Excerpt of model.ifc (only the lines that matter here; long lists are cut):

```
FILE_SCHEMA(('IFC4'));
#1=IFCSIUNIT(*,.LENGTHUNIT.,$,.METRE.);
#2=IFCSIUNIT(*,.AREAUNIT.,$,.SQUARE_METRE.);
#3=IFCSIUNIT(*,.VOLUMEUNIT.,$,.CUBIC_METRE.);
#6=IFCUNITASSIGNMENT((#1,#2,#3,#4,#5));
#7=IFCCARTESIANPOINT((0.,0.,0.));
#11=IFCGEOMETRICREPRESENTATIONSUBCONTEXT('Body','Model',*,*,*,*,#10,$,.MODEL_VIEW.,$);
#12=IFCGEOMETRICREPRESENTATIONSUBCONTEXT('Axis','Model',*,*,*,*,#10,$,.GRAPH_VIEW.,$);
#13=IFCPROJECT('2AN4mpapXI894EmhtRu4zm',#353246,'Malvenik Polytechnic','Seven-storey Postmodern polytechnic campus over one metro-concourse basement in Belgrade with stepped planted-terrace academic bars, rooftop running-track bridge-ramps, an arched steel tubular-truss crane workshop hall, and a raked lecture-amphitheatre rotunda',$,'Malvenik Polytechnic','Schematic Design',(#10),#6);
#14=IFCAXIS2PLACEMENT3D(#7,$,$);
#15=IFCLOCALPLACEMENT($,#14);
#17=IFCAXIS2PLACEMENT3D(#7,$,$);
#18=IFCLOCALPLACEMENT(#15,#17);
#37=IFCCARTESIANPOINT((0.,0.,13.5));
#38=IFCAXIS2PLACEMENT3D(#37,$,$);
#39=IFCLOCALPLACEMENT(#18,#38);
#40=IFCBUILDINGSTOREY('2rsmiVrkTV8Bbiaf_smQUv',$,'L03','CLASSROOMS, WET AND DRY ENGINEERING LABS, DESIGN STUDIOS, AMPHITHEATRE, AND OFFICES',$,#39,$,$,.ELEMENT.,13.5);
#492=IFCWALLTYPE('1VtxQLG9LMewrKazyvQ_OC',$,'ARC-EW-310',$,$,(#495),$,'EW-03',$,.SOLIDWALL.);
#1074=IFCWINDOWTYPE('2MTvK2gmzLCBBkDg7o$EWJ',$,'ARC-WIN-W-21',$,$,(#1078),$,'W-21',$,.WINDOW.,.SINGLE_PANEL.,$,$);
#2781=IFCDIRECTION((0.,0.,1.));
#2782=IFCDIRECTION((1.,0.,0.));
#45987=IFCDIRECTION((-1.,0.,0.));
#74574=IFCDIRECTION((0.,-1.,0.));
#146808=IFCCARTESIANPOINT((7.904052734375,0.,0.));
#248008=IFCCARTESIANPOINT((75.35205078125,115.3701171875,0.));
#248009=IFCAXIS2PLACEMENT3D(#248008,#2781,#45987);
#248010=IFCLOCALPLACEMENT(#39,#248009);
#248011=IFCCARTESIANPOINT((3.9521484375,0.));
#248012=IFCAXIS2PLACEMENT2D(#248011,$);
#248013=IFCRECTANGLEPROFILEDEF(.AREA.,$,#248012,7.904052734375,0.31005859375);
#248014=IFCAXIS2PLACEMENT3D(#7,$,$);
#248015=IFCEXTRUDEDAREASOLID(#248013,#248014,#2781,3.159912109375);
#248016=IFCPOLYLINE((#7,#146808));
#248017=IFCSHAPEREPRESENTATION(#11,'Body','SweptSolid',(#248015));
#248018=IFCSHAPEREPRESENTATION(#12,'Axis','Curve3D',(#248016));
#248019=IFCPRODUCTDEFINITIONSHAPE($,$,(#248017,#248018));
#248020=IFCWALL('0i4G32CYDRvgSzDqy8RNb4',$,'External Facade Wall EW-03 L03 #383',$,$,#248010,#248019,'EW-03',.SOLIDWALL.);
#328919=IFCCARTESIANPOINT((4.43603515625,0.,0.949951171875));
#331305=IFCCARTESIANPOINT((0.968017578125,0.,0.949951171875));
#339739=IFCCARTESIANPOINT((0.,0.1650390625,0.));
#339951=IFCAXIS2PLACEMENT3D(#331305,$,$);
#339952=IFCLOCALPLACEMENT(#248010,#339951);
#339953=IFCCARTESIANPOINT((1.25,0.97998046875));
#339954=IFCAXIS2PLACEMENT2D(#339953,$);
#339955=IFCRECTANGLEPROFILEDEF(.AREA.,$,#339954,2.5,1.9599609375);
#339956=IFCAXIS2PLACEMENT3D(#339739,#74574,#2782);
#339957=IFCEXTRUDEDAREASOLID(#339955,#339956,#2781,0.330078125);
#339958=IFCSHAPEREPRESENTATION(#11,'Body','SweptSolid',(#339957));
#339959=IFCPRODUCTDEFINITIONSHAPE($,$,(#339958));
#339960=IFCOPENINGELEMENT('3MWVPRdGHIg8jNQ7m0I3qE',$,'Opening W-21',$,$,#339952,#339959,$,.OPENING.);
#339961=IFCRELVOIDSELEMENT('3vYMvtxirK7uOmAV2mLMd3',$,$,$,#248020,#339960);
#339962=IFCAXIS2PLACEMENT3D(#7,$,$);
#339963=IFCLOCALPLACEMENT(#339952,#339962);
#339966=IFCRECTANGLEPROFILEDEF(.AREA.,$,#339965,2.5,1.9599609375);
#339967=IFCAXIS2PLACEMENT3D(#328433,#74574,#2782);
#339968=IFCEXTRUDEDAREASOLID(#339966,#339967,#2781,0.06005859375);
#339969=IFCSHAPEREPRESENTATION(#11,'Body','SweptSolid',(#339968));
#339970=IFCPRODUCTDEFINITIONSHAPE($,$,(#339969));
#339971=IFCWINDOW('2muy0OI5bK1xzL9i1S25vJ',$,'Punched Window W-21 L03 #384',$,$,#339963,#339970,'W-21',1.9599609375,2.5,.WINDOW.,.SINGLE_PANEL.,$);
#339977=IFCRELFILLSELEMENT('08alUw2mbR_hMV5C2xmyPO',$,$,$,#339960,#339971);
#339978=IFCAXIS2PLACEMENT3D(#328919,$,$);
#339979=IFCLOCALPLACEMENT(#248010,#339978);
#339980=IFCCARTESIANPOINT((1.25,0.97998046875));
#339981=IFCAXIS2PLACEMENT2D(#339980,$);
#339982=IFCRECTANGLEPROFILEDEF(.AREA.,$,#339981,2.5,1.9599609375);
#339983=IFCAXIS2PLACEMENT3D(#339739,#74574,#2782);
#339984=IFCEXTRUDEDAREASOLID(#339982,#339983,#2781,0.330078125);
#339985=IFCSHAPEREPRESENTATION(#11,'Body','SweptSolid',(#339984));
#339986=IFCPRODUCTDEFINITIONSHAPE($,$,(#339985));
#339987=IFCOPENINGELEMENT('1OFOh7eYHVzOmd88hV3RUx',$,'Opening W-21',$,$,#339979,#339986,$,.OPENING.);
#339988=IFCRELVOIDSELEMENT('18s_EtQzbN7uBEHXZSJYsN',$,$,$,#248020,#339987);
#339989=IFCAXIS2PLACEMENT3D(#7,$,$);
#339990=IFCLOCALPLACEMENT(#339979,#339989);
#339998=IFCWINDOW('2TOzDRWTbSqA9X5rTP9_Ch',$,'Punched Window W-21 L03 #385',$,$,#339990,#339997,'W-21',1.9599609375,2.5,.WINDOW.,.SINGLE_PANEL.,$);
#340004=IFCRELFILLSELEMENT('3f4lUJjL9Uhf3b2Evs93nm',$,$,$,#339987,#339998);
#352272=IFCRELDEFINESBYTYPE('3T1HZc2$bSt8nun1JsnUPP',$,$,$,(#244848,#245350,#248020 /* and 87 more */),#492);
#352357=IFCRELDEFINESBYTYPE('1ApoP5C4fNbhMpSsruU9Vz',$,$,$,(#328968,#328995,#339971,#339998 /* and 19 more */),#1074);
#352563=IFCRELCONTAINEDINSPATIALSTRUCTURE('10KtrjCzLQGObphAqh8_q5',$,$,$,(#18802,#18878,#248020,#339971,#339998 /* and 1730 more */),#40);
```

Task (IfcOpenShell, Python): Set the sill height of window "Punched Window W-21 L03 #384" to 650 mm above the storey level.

```python
import numpy as np
import ifcopenshell
import ifcopenshell.api.geometry
import ifcopenshell.geom
import ifcopenshell.util.element
import ifcopenshell.util.placement
import ifcopenshell.util.shape
import ifcopenshell.util.unit

model = ifcopenshell.open("model.ifc")
unit_scale = ifcopenshell.util.unit.calculate_unit_scale(model)

window = model.by_guid("2muy0OI5bK1xzL9i1S25vJ")
opening = window.FillsVoids[0].RelatingOpeningElement
storey = ifcopenshell.util.element.get_container(window, ifc_class="IfcBuildingStorey")
level = ifcopenshell.util.placement.get_local_placement(storey.ObjectPlacement)[2, 3]

# The opening's origin need not be at the sill, so measure its lowest point.
shape = ifcopenshell.geom.create_shape(ifcopenshell.geom.settings(), opening)
bottom = ifcopenshell.util.shape.get_shape_bottom_elevation(shape, shape.geometry) / unit_scale
dz = level + 0.65 / unit_scale - bottom

shift = np.array([0.0, 0.0, dz])
# The window is placed relative to its opening, so it follows when the opening moves.
matrix = ifcopenshell.util.placement.get_local_placement(opening.ObjectPlacement)
matrix[:3, 3] += shift
ifcopenshell.api.geometry.edit_object_placement(
    model, product=opening, matrix=matrix, is_si=False, should_transform_children=True
)

print(f"moved by {dz * unit_scale:+.3f} m")

model.write("model_rev.ifc")
```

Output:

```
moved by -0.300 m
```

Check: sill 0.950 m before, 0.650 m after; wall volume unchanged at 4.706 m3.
